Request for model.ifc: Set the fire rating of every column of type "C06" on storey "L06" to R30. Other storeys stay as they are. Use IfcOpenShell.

First a look at what the model holds.

```python
import ifcopenshell
import ifcopenshell.util.element

model = ifcopenshell.open("model.ifc")
print(model.schema)
storey = next(s for s in model.by_type("IfcBuildingStorey") if s.Name == "L06")
columns = [e for e in ifcopenshell.util.element.get_decomposition(storey) if e.is_a("IfcColumn")]
seen = {}
for e in columns:
    element_type = ifcopenshell.util.element.get_type(e)
    key = (element_type.Name if element_type != e and element_type else None, ifcopenshell.util.element.get_pset(e, "Pset_ColumnCommon", "FireRating"))
    seen[key] = seen.get(key, 0) + 1
for (name, value), count in sorted(seen.items(), key=str):
    print(count, "x", name, "|", value)
```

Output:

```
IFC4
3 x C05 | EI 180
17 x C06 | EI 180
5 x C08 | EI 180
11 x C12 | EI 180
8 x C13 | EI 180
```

```python
import ifcopenshell
import ifcopenshell.api.pset
import ifcopenshell.util.element

model = ifcopenshell.open("model.ifc")

storey = next(s for s in model.by_type("IfcBuildingStorey") if s.Name == "L06")
columns = [e for e in ifcopenshell.util.element.get_decomposition(storey) if e.is_a("IfcColumn")]

count = 0
for e in columns:
    element_type = ifcopenshell.util.element.get_type(e)
    if element_type in (None, e) or element_type.Name != "C06":
        continue
    # add_pset returns the element's existing set when there is one.
    pset = ifcopenshell.api.pset.add_pset(model, product=e, name="Pset_ColumnCommon")
    ifcopenshell.api.pset.edit_pset(model, pset=pset, properties={"FireRating": "R30"})
    count += 1

print(count, "columns updated")

model.write("model_updated.ifc")
```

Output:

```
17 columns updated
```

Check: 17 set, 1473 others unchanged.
